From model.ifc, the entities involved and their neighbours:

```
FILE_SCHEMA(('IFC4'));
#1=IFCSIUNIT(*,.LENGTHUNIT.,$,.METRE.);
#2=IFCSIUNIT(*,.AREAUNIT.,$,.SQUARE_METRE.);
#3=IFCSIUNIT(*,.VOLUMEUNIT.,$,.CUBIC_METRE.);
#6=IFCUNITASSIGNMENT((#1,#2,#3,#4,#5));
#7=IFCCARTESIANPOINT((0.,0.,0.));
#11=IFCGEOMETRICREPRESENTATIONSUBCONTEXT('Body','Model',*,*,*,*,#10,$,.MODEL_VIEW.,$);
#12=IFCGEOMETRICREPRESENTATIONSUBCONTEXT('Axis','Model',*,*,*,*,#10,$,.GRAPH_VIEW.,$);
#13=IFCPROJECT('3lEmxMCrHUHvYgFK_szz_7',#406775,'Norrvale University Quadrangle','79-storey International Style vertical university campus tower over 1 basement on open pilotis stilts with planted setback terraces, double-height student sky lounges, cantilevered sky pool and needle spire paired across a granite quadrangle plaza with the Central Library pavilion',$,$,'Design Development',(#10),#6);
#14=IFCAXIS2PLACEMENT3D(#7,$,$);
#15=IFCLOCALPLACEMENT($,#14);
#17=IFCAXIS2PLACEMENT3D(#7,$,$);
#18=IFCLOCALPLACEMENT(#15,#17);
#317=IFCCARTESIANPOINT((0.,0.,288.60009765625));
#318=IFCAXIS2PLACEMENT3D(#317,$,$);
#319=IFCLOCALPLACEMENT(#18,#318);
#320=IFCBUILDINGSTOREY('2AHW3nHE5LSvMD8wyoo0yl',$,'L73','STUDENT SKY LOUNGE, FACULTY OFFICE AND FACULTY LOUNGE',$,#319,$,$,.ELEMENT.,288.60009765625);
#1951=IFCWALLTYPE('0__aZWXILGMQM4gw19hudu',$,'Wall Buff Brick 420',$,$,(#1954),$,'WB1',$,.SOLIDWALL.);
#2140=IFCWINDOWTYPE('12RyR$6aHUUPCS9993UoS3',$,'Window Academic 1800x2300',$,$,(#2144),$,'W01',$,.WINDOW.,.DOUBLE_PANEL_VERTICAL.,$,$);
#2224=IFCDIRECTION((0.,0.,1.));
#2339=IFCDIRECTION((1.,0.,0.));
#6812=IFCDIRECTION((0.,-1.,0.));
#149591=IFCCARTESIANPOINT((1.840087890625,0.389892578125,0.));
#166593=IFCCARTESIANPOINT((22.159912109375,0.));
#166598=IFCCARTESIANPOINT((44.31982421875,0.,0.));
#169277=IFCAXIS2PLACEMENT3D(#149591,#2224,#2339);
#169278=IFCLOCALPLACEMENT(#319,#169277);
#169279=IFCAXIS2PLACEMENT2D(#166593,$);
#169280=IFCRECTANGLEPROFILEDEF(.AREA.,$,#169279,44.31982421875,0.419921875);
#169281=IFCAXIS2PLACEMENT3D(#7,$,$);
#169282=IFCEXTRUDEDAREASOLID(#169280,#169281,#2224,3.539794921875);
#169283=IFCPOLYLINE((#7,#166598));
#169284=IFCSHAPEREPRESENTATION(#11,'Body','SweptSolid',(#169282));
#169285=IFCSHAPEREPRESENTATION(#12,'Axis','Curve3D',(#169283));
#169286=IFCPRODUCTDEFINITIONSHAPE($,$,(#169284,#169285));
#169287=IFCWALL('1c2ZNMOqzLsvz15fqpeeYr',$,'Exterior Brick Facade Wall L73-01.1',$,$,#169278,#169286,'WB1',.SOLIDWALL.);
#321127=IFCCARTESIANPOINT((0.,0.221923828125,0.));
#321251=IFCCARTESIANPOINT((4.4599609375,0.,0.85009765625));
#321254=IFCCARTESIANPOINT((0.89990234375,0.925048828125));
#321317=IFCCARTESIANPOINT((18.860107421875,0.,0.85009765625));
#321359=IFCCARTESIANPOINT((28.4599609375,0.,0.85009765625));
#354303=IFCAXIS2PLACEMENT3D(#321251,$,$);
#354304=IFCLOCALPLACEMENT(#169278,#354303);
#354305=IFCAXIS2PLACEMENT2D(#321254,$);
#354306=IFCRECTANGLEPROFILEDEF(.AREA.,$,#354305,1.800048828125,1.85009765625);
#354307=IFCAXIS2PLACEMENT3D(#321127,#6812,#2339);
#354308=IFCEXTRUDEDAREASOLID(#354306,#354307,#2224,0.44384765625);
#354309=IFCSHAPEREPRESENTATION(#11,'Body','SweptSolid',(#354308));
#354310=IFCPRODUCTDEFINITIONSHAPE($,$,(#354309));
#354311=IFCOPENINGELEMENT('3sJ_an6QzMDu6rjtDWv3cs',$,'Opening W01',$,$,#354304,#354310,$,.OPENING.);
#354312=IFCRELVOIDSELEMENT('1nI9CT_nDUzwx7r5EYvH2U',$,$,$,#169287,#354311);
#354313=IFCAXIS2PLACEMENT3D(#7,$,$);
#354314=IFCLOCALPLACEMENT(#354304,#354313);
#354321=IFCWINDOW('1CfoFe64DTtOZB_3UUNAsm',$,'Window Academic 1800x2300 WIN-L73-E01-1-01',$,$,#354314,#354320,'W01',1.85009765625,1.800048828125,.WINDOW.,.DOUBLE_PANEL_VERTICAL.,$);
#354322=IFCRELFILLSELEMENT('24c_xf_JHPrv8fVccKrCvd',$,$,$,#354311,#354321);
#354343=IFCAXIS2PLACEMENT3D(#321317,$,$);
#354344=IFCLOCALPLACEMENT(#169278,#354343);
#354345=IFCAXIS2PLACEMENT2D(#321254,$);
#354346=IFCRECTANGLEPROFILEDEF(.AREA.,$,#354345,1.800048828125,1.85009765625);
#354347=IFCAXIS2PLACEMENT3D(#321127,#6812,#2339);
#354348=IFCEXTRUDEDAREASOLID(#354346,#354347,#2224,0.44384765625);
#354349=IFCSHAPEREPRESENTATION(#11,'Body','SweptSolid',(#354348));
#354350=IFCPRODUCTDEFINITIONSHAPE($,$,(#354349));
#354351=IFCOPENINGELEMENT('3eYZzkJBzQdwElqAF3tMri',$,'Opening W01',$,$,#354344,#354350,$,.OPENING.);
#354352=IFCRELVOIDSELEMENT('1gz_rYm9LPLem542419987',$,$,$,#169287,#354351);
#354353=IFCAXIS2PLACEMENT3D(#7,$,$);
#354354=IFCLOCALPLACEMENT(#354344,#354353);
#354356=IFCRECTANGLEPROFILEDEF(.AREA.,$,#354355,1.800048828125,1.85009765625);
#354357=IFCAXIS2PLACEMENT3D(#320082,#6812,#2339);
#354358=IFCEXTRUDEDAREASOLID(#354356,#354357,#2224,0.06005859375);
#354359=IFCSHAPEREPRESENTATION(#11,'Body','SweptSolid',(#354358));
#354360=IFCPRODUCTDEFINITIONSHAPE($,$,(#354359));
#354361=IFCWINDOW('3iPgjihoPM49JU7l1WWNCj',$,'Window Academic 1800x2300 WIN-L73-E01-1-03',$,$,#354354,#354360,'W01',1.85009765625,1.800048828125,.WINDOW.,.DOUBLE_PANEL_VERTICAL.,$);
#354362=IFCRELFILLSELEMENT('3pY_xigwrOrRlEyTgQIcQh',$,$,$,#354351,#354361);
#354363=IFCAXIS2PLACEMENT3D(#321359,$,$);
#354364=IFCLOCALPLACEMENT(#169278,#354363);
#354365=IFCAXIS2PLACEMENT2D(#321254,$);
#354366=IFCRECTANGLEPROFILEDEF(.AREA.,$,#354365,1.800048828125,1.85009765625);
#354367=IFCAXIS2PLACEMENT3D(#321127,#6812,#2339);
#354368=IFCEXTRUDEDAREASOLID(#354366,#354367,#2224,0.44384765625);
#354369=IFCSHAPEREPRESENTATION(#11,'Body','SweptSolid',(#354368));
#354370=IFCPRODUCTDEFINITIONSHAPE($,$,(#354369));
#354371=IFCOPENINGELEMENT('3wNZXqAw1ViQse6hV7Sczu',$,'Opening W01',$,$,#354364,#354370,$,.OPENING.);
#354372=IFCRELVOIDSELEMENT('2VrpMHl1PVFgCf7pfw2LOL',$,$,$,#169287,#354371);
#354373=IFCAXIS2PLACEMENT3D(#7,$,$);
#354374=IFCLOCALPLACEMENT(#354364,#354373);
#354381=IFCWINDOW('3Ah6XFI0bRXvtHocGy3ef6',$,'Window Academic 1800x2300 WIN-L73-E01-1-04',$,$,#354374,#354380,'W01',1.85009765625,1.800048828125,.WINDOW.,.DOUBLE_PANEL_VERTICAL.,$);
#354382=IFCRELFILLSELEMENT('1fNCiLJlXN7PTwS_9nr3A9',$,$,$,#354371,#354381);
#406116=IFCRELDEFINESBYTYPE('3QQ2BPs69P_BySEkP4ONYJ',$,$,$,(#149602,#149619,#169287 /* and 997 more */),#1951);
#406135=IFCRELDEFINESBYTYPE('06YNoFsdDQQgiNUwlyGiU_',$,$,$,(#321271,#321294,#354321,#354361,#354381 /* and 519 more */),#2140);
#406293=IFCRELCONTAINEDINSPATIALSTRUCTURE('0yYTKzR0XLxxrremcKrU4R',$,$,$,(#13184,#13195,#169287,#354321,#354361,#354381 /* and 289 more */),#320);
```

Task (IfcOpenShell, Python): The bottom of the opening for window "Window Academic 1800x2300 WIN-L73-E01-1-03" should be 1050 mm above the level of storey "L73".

```python
import numpy as np
import ifcopenshell
import ifcopenshell.api.geometry
import ifcopenshell.geom
import ifcopenshell.util.element
import ifcopenshell.util.placement
import ifcopenshell.util.shape
import ifcopenshell.util.unit

model = ifcopenshell.open("model.ifc")
unit_scale = ifcopenshell.util.unit.calculate_unit_scale(model)

window = model.by_guid("3iPgjihoPM49JU7l1WWNCj")
opening = window.FillsVoids[0].RelatingOpeningElement
storey = ifcopenshell.util.element.get_container(window, ifc_class="IfcBuildingStorey")
level = ifcopenshell.util.placement.get_local_placement(storey.ObjectPlacement)[2, 3]

# The opening's origin need not be at the sill, so measure its lowest point.
shape = ifcopenshell.geom.create_shape(ifcopenshell.geom.settings(), opening)
bottom = ifcopenshell.util.shape.get_shape_bottom_elevation(shape, shape.geometry) / unit_scale
dz = level + 1.05 / unit_scale - bottom

shift = np.array([0.0, 0.0, dz])
# The window is placed relative to its opening, so it follows when the opening moves.
matrix = ifcopenshell.util.placement.get_local_placement(opening.ObjectPlacement)
matrix[:3, 3] += shift
ifcopenshell.api.geometry.edit_object_placement(
    model, product=opening, matrix=matrix, is_si=False, should_transform_children=True
)

print(f"moved by {dz * unit_scale:+.3f} m")

model.write("model_updated.ifc")
```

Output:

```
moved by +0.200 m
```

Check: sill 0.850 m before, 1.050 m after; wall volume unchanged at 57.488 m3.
